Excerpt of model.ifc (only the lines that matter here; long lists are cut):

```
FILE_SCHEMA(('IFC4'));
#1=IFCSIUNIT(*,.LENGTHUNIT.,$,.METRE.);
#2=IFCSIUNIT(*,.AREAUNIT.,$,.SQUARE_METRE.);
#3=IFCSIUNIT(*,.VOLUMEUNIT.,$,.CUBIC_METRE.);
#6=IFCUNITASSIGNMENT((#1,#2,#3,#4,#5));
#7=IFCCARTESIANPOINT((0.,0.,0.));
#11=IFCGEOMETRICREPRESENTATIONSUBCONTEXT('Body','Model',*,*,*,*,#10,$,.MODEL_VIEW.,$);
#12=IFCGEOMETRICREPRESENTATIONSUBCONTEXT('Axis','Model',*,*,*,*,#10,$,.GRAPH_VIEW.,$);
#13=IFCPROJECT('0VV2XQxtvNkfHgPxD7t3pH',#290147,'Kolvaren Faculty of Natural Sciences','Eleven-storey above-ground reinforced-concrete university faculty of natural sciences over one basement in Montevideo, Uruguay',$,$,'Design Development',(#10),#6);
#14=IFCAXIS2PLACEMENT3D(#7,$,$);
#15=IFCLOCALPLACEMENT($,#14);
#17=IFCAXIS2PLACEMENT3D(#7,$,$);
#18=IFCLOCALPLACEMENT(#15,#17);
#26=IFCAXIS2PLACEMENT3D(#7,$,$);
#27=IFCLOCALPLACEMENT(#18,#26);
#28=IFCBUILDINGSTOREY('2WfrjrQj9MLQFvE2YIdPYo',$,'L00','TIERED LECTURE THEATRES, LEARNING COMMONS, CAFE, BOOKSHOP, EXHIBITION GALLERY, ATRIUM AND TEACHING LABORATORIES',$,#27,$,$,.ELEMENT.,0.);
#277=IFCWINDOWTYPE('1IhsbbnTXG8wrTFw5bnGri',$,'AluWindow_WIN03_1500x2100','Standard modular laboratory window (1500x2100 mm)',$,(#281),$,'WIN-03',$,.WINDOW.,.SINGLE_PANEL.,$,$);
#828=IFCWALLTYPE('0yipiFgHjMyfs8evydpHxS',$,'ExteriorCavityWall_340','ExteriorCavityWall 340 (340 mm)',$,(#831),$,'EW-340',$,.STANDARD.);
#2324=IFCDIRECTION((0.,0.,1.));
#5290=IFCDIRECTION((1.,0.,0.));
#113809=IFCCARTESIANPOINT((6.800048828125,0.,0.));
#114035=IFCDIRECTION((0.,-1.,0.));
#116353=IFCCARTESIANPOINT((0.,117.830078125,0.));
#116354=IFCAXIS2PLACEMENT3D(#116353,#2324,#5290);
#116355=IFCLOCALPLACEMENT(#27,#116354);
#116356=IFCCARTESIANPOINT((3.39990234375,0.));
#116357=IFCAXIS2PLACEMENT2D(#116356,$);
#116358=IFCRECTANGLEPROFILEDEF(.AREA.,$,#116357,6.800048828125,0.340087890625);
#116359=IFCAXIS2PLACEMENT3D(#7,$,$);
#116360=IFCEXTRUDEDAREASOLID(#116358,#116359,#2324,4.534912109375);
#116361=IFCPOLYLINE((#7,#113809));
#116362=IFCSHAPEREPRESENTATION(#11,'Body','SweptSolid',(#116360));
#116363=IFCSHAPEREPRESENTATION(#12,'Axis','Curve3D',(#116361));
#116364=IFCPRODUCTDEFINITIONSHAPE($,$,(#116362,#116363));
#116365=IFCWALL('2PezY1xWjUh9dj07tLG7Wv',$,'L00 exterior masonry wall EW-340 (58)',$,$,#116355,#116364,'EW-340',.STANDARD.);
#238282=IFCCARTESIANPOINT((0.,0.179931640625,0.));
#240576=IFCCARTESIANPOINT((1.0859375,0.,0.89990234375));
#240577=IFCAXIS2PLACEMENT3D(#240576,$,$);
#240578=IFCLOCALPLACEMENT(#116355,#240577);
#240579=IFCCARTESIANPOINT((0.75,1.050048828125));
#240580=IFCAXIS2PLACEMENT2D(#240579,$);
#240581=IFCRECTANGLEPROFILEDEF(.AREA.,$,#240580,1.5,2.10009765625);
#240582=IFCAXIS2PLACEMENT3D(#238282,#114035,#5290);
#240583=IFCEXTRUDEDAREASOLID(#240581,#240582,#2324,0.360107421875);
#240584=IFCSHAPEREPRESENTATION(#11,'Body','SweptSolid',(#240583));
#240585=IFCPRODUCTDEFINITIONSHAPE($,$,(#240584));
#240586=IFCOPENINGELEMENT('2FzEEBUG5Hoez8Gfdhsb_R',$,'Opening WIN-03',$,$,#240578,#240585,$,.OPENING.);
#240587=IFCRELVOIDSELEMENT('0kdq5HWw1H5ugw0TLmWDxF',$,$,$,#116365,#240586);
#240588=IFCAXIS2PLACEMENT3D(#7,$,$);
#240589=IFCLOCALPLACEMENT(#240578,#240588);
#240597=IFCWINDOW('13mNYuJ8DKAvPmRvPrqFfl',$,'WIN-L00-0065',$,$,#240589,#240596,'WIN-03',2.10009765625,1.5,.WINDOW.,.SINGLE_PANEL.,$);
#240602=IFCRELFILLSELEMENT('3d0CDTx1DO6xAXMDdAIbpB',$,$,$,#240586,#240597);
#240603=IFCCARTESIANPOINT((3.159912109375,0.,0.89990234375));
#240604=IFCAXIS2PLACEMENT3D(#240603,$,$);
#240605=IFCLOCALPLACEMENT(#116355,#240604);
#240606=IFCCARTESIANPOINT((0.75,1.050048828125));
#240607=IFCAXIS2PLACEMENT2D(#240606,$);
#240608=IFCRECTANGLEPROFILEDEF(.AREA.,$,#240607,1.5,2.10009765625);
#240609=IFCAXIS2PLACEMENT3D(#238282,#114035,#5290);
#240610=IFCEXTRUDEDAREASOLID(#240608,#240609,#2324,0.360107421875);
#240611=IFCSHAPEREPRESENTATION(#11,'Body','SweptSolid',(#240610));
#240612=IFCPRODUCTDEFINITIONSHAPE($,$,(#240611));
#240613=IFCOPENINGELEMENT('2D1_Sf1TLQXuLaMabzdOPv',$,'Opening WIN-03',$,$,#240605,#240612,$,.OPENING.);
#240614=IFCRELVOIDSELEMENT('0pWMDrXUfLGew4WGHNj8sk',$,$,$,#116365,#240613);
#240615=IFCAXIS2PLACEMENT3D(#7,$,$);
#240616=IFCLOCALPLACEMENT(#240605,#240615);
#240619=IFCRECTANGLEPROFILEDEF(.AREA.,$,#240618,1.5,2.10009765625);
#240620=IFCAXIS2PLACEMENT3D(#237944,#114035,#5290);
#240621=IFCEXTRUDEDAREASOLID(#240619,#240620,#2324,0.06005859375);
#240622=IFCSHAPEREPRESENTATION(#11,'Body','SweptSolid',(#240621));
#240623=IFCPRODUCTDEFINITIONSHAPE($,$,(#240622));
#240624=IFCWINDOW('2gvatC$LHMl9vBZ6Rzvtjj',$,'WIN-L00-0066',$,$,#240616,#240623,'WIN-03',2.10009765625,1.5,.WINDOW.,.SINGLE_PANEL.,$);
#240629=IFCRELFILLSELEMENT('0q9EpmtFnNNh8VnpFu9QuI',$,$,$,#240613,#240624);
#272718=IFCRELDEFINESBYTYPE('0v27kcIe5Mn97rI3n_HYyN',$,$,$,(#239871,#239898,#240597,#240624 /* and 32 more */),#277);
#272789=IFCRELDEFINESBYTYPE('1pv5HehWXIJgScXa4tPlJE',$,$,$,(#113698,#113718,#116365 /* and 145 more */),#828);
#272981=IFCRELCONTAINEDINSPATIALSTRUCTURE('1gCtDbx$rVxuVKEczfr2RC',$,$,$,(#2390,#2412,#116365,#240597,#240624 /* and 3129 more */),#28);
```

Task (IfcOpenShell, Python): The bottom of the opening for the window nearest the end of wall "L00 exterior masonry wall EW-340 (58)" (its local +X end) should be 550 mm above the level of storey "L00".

```python
import numpy as np
import ifcopenshell
import ifcopenshell.api.geometry
import ifcopenshell.geom
import ifcopenshell.util.element
import ifcopenshell.util.placement
import ifcopenshell.util.shape
import ifcopenshell.util.unit

model = ifcopenshell.open("model.ifc")
unit_scale = ifcopenshell.util.unit.calculate_unit_scale(model)

window = model.by_guid("2gvatC$LHMl9vBZ6Rzvtjj")
opening = window.FillsVoids[0].RelatingOpeningElement
storey = ifcopenshell.util.element.get_container(window, ifc_class="IfcBuildingStorey")
level = ifcopenshell.util.placement.get_local_placement(storey.ObjectPlacement)[2, 3]

# The opening's origin need not be at the sill, so measure its lowest point.
shape = ifcopenshell.geom.create_shape(ifcopenshell.geom.settings(), opening)
bottom = ifcopenshell.util.shape.get_shape_bottom_elevation(shape, shape.geometry) / unit_scale
dz = level + 0.55 / unit_scale - bottom

shift = np.array([0.0, 0.0, dz])
# The window is placed relative to its opening, so it follows when the opening moves.
matrix = ifcopenshell.util.placement.get_local_placement(opening.ObjectPlacement)
matrix[:3, 3] += shift
ifcopenshell.api.geometry.edit_object_placement(
    model, product=opening, matrix=matrix, is_si=False, should_transform_children=True
)

print(f"moved by {dz * unit_scale:+.3f} m")

model.write("model-out.ifc")
```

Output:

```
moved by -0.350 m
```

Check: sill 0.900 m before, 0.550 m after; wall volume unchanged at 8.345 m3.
